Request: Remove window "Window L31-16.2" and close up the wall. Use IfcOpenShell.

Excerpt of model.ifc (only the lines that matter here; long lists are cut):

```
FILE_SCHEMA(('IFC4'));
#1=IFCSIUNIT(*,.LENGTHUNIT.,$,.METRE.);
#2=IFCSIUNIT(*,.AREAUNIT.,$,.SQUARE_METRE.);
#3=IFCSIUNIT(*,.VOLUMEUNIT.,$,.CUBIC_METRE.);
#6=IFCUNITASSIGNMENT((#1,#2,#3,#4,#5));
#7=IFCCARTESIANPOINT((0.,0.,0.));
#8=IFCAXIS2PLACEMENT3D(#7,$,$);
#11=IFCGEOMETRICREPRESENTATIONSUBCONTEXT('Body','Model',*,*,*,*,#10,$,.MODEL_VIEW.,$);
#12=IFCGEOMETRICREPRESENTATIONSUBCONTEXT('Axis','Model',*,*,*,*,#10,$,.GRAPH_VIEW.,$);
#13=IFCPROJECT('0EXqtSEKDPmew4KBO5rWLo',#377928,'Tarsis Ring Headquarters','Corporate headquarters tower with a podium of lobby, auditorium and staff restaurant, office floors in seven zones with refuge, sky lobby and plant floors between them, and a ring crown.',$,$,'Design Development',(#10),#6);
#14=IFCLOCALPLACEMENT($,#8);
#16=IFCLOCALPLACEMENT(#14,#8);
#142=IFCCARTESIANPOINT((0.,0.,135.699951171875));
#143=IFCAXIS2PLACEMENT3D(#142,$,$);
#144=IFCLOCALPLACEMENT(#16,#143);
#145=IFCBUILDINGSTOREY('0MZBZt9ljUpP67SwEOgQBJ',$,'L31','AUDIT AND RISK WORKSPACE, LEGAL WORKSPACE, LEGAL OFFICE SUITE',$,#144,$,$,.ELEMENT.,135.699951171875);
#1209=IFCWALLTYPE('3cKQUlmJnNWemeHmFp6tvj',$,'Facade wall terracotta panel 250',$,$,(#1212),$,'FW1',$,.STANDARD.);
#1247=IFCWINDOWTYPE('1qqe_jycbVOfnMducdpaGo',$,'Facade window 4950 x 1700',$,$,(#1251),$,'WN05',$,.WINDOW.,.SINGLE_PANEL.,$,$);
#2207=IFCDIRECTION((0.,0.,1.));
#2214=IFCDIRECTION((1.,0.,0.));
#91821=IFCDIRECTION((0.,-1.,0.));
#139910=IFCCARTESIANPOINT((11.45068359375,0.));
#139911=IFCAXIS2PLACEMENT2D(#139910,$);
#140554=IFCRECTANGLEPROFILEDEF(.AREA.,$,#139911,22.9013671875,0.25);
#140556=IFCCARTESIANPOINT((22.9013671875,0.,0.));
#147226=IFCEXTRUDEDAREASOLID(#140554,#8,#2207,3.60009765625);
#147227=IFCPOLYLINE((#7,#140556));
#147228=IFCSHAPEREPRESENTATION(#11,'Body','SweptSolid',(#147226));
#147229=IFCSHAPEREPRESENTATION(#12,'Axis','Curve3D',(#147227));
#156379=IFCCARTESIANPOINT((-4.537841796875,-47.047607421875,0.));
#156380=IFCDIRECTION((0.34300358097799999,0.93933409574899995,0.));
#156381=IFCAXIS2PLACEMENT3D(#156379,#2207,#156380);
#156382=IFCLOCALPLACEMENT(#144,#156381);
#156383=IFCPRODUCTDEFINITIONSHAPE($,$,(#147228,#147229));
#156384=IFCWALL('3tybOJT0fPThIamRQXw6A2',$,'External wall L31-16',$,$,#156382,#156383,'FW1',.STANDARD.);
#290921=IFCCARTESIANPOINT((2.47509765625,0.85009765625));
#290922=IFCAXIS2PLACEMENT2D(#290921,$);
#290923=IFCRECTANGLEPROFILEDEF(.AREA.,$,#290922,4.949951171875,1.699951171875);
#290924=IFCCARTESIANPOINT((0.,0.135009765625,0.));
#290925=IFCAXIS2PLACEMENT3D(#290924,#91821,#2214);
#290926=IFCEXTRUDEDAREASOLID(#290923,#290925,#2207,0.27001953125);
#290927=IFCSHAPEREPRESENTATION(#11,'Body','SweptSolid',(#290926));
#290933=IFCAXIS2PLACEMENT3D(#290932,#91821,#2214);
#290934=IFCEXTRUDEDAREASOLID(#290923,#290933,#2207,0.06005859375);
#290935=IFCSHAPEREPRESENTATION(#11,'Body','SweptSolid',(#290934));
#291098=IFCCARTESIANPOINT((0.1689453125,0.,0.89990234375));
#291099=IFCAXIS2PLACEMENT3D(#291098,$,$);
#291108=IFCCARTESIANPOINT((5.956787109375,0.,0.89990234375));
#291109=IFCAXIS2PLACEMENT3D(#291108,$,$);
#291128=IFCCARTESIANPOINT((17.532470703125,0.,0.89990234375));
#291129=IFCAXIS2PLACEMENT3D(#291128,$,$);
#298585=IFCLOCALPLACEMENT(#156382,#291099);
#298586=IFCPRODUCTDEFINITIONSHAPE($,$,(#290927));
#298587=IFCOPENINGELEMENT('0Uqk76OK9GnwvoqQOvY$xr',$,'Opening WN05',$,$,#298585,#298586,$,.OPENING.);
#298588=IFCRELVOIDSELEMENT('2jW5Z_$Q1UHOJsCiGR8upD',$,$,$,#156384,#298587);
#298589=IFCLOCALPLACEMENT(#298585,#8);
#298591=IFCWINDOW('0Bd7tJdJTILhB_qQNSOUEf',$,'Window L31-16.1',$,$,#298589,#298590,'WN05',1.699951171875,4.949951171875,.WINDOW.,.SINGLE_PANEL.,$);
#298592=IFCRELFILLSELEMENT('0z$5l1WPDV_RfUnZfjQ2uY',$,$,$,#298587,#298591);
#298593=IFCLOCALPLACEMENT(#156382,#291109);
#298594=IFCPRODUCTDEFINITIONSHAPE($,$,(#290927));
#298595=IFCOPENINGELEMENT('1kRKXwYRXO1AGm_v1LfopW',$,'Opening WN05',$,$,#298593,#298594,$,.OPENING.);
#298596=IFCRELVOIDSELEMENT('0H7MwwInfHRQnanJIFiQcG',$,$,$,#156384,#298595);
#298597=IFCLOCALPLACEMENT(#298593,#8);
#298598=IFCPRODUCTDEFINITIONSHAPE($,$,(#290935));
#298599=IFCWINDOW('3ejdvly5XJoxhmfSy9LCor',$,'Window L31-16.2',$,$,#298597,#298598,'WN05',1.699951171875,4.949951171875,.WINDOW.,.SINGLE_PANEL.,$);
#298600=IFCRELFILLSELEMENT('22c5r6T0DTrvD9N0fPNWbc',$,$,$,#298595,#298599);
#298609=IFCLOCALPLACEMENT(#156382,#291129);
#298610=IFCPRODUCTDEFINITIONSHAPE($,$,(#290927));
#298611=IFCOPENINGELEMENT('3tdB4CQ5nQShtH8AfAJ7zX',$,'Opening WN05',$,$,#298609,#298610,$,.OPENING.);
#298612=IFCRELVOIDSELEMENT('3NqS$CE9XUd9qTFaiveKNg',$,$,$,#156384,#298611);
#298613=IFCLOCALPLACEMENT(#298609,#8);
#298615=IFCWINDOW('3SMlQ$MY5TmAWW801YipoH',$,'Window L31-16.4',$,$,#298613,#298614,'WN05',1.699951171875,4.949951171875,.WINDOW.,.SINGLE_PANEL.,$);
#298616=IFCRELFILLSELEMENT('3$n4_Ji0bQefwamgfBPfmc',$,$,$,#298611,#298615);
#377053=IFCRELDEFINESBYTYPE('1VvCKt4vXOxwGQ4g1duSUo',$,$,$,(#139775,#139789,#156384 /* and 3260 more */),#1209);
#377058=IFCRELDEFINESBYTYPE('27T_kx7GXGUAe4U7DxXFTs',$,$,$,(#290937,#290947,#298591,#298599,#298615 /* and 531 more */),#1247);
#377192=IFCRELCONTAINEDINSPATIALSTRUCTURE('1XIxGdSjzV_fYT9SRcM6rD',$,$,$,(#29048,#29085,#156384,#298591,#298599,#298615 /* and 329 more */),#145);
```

```python
import ifcopenshell
import ifcopenshell.api.feature
import ifcopenshell.api.root
import ifcopenshell.geom
import ifcopenshell.util.shape

model = ifcopenshell.open("model.ifc")
settings = ifcopenshell.geom.settings()


def volume(element):
    """Net volume in cubic metres, openings subtracted."""
    shape = ifcopenshell.geom.create_shape(settings, element)
    return ifcopenshell.util.shape.get_volume(shape.geometry)


window = model.by_id(298599)
opening = window.FillsVoids[0].RelatingOpeningElement
wall = opening.VoidsElements[0].RelatingBuildingElement
before = volume(wall)

ifcopenshell.api.root.remove_product(model, product=window)
ifcopenshell.api.feature.remove_feature(model, feature=opening)

after = volume(wall)

print(f"wall volume {before:.3f} -> {after:.3f} m3")

model.write("model_edited.ifc")
```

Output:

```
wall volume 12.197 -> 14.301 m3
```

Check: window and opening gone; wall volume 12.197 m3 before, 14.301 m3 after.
